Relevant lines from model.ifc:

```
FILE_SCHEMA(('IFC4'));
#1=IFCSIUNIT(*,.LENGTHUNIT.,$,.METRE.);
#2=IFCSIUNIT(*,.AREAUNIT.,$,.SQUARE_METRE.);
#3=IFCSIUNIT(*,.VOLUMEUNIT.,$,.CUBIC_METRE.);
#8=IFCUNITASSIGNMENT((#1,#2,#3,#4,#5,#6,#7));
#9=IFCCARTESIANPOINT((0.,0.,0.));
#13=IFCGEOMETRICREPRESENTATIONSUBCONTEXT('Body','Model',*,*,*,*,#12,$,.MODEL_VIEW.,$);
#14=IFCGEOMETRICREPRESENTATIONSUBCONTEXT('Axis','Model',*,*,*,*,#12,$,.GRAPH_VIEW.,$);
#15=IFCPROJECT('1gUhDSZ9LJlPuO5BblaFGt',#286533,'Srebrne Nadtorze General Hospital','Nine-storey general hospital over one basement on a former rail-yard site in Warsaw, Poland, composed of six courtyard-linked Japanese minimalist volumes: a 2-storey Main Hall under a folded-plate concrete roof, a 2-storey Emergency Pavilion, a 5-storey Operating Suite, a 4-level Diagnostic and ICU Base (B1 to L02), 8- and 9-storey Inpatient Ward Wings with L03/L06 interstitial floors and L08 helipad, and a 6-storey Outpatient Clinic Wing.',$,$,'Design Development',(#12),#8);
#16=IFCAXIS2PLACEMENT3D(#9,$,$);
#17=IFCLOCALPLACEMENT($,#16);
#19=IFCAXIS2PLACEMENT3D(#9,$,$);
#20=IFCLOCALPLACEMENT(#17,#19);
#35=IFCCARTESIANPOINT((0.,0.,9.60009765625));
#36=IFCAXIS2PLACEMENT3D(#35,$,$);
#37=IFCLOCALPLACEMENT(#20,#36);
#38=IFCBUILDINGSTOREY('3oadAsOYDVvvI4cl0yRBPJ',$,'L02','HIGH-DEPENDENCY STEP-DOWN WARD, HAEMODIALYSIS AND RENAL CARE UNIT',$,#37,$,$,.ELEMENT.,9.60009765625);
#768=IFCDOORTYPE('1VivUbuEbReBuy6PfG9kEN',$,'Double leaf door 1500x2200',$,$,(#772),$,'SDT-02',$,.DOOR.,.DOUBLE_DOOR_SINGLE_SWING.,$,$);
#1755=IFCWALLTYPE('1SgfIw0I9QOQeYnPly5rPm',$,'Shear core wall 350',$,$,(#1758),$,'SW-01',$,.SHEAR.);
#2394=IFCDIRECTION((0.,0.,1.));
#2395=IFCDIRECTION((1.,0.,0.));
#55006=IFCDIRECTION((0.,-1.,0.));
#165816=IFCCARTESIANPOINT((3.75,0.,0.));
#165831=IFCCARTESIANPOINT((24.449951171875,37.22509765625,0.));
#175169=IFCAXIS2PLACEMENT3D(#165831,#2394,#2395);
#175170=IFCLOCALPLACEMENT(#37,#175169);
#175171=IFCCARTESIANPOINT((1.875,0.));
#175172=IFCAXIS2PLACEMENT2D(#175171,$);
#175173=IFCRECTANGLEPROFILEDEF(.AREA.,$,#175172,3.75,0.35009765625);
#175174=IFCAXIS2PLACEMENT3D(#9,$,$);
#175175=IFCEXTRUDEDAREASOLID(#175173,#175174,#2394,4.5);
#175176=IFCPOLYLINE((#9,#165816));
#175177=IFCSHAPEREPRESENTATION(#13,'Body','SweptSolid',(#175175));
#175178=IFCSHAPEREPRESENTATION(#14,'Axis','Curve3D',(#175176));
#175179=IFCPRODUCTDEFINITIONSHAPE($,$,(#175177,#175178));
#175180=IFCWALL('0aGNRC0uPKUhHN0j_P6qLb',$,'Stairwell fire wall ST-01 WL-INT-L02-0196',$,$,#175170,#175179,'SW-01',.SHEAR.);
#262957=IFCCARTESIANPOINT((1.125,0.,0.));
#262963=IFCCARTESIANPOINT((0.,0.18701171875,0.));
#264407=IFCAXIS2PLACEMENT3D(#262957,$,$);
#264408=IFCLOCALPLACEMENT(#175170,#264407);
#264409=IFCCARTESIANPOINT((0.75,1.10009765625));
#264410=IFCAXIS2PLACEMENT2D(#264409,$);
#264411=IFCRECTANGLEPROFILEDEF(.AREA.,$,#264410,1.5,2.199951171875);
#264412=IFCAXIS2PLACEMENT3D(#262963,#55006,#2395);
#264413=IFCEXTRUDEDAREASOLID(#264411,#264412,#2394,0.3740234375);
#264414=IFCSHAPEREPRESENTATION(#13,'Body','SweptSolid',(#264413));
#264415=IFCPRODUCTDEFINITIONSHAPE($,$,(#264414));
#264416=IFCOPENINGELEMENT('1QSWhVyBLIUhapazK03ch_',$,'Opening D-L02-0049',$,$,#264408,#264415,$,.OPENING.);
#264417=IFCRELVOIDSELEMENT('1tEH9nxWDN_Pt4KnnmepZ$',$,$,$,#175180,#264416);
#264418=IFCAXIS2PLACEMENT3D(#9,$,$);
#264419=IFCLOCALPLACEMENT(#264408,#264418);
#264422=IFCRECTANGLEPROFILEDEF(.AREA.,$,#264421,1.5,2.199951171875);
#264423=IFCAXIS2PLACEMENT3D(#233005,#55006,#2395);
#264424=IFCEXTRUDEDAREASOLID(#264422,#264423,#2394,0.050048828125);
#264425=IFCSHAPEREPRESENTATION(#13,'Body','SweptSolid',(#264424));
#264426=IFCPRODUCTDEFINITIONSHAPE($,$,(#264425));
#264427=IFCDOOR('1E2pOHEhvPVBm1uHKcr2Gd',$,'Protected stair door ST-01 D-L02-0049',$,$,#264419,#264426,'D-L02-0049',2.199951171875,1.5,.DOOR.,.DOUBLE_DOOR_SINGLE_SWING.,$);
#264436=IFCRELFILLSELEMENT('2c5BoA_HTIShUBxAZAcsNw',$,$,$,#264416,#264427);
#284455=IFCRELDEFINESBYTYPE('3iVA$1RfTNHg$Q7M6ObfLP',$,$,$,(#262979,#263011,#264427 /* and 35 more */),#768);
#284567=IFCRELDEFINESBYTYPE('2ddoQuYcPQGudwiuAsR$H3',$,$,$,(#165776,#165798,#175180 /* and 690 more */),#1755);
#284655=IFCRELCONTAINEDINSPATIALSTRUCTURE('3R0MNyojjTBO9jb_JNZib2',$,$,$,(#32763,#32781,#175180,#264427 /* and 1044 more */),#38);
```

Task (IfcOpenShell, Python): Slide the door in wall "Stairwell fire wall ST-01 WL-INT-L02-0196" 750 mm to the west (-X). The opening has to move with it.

```python
import ifcopenshell
import ifcopenshell.api.geometry
import ifcopenshell.util.placement
import ifcopenshell.util.unit

model = ifcopenshell.open("model.ifc")
unit_scale = ifcopenshell.util.unit.calculate_unit_scale(model)

door = model.by_guid("1E2pOHEhvPVBm1uHKcr2Gd")
opening = door.FillsVoids[0].RelatingOpeningElement
wall = opening.VoidsElements[0].RelatingBuildingElement

wall_matrix = ifcopenshell.util.placement.get_local_placement(wall.ObjectPlacement)
shift = wall_matrix[:3, 0] * -0.75 / unit_scale
before = ifcopenshell.util.placement.get_local_placement(door.ObjectPlacement)[:3, 3].copy()

# The door is placed relative to its opening, so it follows when the opening moves.
matrix = ifcopenshell.util.placement.get_local_placement(opening.ObjectPlacement)
matrix[:3, 3] += shift
ifcopenshell.api.geometry.edit_object_placement(
    model, product=opening, matrix=matrix, is_si=False, should_transform_children=True
)

after = ifcopenshell.util.placement.get_local_placement(door.ObjectPlacement)[:3, 3]
print("door moved by", (after - before).round(3) + 0.0)

model.write("model_rev.ifc")
```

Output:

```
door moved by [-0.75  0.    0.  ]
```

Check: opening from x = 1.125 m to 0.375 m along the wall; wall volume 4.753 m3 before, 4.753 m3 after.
